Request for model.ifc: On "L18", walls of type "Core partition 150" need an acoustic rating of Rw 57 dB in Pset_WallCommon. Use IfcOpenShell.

First a look at what the model holds.

```python
import ifcopenshell
import ifcopenshell.util.element

model = ifcopenshell.open("model.ifc")
print(model.schema)
storey = next(s for s in model.by_type("IfcBuildingStorey") if s.Name == "L18")
walls = [e for e in ifcopenshell.util.element.get_decomposition(storey) if e.is_a("IfcWall")]
seen = {}
for e in walls:
    element_type = ifcopenshell.util.element.get_type(e)
    key = (element_type.Name if element_type != e and element_type else None, ifcopenshell.util.element.get_pset(e, "Pset_WallCommon", "AcousticRating"))
    seen[key] = seen.get(key, 0) + 1
for (name, value), count in sorted(seen.items(), key=str):
    print(count, "x", name, "|", value)
```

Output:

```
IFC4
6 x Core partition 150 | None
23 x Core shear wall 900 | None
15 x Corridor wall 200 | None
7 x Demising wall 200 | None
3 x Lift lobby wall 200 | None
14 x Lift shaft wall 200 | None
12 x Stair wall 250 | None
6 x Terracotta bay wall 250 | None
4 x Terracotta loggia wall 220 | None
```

```python
import ifcopenshell
import ifcopenshell.api.pset
import ifcopenshell.util.element

model = ifcopenshell.open("model.ifc")

storey = next(s for s in model.by_type("IfcBuildingStorey") if s.Name == "L18")
walls = [e for e in ifcopenshell.util.element.get_decomposition(storey) if e.is_a("IfcWall")]

count = 0
for e in walls:
    element_type = ifcopenshell.util.element.get_type(e)
    if element_type in (None, e) or element_type.Name != "Core partition 150":
        continue
    found = ifcopenshell.util.element.get_pset(e, "Pset_WallCommon", should_inherit=False)
    if found:
        pset = model.by_id(found["id"])
        if len(ifcopenshell.util.element.get_elements_by_pset(pset)) > 1:
            pset = ifcopenshell.api.pset.unshare_pset(model, products=[e], pset=pset)[0]
    else:
        pset = ifcopenshell.api.pset.add_pset(model, product=e, name="Pset_WallCommon")
    ifcopenshell.api.pset.edit_pset(model, pset=pset, properties={"AcousticRating": "Rw 57 dB"})
    count += 1

print(count, "walls updated")

model.write("model_updated.ifc")
```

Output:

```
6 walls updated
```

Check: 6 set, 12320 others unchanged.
